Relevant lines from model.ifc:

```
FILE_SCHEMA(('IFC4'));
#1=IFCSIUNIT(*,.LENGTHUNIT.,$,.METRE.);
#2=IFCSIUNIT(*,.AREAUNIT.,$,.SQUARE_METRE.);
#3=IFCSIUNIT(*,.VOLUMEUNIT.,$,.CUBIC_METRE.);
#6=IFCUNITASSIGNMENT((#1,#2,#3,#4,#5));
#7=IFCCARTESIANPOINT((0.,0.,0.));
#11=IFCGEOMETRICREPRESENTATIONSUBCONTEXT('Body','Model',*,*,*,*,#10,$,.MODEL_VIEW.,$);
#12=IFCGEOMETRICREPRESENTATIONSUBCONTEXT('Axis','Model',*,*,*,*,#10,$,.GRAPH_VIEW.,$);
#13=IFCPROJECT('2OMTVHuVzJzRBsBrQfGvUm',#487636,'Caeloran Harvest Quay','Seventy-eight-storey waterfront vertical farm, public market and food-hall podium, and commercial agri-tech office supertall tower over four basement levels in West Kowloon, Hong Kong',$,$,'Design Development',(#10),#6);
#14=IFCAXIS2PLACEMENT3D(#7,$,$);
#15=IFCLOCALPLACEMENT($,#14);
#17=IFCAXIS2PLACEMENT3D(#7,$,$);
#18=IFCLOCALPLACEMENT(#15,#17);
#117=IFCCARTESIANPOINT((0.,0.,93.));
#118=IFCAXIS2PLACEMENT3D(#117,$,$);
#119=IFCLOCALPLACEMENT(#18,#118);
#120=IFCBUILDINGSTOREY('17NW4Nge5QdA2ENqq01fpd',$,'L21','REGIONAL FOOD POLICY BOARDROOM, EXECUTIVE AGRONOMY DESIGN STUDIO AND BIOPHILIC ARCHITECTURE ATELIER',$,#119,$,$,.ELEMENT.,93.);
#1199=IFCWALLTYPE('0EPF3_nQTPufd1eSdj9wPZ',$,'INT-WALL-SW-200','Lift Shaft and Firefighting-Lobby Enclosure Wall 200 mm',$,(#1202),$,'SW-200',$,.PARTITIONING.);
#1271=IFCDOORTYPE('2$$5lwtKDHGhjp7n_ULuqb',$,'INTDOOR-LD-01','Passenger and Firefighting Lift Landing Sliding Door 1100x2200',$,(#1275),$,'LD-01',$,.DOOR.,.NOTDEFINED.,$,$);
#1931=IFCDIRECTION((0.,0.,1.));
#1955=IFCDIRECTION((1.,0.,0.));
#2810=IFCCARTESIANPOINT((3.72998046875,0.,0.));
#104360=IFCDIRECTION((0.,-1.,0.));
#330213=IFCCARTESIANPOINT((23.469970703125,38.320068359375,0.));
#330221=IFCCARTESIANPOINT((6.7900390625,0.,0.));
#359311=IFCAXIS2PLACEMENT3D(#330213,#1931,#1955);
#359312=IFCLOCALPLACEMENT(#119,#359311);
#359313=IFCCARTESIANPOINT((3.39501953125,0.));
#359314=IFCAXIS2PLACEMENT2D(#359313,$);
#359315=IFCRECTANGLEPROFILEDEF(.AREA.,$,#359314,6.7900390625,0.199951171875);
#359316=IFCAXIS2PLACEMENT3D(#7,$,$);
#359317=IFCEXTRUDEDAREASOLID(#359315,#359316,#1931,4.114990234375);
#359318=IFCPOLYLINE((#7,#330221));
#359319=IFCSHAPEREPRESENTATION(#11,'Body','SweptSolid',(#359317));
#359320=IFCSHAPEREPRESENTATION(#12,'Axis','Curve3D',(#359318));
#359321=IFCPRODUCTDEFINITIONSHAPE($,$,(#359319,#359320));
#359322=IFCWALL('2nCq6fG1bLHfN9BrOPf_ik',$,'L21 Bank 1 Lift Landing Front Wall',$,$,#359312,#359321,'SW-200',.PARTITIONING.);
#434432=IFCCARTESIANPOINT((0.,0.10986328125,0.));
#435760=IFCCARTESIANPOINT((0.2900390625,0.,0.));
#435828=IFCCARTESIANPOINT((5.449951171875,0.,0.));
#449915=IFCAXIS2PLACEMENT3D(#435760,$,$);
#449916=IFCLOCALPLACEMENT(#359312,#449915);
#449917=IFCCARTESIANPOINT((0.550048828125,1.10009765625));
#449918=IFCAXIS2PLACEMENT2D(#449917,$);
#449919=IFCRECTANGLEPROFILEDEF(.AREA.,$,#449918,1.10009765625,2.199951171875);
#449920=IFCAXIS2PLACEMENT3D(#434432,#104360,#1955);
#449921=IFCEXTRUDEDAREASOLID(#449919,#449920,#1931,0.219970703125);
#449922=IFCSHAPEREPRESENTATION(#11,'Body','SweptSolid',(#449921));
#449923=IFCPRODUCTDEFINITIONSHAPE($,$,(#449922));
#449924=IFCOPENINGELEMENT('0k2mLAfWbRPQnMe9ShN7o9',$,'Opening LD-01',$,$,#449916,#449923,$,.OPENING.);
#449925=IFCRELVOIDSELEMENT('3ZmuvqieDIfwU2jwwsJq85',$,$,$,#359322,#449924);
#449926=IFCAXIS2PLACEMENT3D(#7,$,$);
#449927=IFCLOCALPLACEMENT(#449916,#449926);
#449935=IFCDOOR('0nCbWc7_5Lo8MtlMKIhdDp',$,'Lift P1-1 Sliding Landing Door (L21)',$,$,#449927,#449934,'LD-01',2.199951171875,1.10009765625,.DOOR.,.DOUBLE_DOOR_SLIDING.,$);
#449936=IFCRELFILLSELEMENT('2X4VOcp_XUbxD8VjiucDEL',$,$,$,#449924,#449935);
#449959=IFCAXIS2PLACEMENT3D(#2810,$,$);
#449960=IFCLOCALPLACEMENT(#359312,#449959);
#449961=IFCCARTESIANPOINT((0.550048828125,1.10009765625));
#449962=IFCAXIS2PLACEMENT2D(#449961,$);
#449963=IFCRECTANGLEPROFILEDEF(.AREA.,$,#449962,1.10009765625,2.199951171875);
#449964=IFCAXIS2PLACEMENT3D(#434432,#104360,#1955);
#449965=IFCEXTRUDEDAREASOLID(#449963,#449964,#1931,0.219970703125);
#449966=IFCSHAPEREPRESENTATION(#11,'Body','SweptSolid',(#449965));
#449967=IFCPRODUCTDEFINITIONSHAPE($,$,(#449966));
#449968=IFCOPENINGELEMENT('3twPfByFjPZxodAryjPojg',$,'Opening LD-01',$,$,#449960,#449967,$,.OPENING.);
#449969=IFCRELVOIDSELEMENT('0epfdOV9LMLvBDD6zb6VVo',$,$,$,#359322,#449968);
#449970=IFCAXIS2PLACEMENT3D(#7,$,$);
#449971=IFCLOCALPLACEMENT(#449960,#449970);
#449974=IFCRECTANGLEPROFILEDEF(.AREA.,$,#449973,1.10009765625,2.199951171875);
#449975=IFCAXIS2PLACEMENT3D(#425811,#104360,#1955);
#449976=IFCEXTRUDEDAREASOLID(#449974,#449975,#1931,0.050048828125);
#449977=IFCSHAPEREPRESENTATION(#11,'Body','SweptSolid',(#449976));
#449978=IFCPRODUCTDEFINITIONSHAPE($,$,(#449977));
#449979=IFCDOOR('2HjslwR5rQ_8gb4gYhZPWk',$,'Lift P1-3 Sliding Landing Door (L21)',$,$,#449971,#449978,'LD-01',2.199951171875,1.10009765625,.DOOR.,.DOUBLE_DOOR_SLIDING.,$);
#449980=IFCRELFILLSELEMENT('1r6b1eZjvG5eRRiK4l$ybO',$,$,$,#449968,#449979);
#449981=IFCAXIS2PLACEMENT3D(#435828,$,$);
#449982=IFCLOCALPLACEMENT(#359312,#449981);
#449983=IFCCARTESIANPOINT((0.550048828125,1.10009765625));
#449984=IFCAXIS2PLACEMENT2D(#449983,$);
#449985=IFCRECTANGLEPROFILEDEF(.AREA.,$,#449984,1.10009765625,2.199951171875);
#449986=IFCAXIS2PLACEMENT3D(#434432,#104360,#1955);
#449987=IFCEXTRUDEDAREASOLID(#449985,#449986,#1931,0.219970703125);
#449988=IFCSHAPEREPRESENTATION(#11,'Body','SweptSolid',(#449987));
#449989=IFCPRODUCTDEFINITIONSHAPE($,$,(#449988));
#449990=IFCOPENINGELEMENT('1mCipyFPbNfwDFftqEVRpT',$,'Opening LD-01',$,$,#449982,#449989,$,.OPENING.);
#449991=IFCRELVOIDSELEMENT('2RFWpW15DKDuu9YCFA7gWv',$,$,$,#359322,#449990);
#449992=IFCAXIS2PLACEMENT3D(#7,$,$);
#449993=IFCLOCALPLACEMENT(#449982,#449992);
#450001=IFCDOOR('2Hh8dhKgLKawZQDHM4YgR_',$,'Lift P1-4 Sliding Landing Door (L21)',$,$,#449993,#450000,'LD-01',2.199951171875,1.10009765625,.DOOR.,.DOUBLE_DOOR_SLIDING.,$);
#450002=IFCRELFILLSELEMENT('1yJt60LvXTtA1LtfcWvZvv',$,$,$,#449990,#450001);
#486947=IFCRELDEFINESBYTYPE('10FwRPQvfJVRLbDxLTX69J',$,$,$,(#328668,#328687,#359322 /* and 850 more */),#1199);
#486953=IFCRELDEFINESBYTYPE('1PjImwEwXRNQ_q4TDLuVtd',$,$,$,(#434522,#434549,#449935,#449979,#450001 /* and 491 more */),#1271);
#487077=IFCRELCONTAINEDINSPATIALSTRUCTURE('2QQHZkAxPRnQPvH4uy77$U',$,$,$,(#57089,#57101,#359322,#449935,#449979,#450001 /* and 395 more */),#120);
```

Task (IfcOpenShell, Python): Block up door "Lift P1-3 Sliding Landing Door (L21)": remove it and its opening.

```python
import ifcopenshell
import ifcopenshell.api.feature
import ifcopenshell.api.root
import ifcopenshell.geom
import ifcopenshell.util.shape

model = ifcopenshell.open("model.ifc")
settings = ifcopenshell.geom.settings()


def volume(element):
    """Net volume in cubic metres, openings subtracted."""
    shape = ifcopenshell.geom.create_shape(settings, element)
    return ifcopenshell.util.shape.get_volume(shape.geometry)


door = model.by_guid("2HjslwR5rQ_8gb4gYhZPWk")
opening = door.FillsVoids[0].RelatingOpeningElement
wall = opening.VoidsElements[0].RelatingBuildingElement
before = volume(wall)

ifcopenshell.api.root.remove_product(model, product=door)
ifcopenshell.api.feature.remove_feature(model, feature=opening)

after = volume(wall)

print(f"wall volume {before:.3f} -> {after:.3f} m3")

model.write("model_updated.ifc")
```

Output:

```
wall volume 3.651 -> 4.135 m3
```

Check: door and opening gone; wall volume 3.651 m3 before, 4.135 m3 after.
